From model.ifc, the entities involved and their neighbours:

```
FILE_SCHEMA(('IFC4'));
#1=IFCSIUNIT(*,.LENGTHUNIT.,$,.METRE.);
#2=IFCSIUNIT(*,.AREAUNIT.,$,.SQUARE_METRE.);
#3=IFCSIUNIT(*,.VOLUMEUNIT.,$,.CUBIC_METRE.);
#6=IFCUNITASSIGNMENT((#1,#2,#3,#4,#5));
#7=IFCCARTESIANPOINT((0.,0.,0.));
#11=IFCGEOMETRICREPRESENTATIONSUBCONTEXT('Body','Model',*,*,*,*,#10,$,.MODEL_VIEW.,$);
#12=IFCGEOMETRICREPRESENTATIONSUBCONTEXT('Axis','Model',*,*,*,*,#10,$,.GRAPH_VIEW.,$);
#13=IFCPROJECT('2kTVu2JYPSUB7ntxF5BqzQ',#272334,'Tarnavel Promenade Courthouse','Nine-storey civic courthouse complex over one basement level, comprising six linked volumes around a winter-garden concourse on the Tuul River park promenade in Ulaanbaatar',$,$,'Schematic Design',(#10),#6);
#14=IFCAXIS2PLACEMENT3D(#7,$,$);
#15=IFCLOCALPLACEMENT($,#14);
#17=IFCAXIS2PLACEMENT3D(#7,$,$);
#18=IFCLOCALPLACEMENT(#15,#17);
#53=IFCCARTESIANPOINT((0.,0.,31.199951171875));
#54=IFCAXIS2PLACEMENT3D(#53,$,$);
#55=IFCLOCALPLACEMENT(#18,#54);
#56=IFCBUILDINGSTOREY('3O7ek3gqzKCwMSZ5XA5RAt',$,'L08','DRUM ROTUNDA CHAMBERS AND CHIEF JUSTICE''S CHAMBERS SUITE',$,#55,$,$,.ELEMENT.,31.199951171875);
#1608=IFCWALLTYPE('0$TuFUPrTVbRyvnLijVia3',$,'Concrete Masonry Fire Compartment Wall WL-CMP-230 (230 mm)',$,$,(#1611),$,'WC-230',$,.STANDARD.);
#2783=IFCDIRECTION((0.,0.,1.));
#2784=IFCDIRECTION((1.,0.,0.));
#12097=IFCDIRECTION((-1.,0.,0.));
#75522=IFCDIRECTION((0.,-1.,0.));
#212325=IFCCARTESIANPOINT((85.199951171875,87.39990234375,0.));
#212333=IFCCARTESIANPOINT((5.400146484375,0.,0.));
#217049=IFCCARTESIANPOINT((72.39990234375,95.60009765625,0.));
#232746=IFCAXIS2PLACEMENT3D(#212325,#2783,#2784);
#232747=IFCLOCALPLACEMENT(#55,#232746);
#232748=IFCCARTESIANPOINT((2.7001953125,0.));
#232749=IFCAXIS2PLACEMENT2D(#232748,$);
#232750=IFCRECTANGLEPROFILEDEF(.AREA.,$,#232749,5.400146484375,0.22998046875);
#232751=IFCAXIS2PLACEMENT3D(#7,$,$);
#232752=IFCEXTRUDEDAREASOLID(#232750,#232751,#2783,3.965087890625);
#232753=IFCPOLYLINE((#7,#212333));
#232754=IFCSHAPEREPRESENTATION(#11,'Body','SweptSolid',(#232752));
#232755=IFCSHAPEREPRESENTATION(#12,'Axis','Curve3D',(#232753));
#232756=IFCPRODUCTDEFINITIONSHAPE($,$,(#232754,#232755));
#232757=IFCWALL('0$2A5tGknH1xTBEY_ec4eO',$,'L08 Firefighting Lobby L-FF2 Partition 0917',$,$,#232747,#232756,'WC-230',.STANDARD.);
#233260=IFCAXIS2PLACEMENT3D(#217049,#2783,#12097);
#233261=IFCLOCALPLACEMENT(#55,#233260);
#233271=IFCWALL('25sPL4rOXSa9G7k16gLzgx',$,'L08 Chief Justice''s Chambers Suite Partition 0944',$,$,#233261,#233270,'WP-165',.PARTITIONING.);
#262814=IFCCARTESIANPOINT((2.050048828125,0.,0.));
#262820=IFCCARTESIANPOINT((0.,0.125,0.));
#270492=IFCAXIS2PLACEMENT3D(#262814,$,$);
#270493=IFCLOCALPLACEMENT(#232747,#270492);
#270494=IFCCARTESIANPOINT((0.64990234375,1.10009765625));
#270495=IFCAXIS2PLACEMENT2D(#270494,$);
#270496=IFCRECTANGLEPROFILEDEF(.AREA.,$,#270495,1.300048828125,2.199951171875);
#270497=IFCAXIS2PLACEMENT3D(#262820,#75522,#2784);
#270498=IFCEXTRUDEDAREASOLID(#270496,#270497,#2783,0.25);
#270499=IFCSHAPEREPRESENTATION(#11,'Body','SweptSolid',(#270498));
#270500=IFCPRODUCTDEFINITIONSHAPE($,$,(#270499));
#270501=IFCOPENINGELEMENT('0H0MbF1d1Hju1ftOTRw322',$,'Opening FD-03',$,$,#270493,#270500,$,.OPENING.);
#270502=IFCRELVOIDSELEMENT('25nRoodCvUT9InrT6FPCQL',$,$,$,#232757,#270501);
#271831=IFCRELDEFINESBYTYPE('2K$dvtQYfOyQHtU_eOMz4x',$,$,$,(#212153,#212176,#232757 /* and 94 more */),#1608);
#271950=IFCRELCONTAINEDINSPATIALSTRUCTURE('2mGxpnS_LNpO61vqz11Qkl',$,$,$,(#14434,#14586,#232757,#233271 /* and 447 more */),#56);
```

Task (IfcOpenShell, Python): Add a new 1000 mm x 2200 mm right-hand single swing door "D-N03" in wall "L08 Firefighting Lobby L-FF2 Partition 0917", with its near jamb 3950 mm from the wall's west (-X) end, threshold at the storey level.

```python
import numpy as np
import ifcopenshell
import ifcopenshell.api.feature
import ifcopenshell.api.geometry
import ifcopenshell.api.root
import ifcopenshell.api.spatial
import ifcopenshell.geom
import ifcopenshell.util.element
import ifcopenshell.util.placement
import ifcopenshell.util.representation
import ifcopenshell.util.shape
import ifcopenshell.util.unit

model = ifcopenshell.open("model.ifc")
unit_scale = ifcopenshell.util.unit.calculate_unit_scale(model)
settings = ifcopenshell.geom.settings()


def volume(element):
    """Net volume in cubic metres, openings subtracted."""
    shape = ifcopenshell.geom.create_shape(settings, element)
    return ifcopenshell.util.shape.get_volume(shape.geometry)


wall = model.by_id(232757)
storey = ifcopenshell.util.element.get_container(wall, ifc_class="IfcBuildingStorey")
context = ifcopenshell.util.representation.get_context(model, "Model", "Body", "MODEL_VIEW")
before = volume(wall)

width, height, from_end, sill = 1, 2.2, 3.95, 0.0  # metres

# The wall runs along its own X axis, and the end named is its -X end.
wall_shape = ifcopenshell.geom.create_shape(settings, wall)
x, y, z = ifcopenshell.util.shape.get_vertices(wall_shape.geometry).T
start = x.min() + from_end
face, thickness = float(y.min()), float(y.max() - y.min())
wall_matrix = ifcopenshell.util.placement.get_local_placement(wall.ObjectPlacement)
level = ifcopenshell.util.placement.get_local_placement(storey.ObjectPlacement)[2, 3]


def in_wall(x, y):
    """Placement at x, y metres in the wall's axes, at sill height."""
    matrix = wall_matrix.copy()
    matrix[:, 3] = wall_matrix @ np.array([x / unit_scale, y / unit_scale, 0.0, 1.0])
    matrix[2, 3] = level + sill / unit_scale
    return matrix


# Opening: a box that overshoots both wall faces by 50 mm.
opening = ifcopenshell.api.root.create_entity(model, ifc_class="IfcOpeningElement", predefined_type="OPENING")
box = ifcopenshell.api.geometry.add_wall_representation(
    model, context=context, length=width, height=height, thickness=thickness + 0.1
)
ifcopenshell.api.geometry.assign_representation(model, product=opening, representation=box)
ifcopenshell.api.geometry.edit_object_placement(model, product=opening, matrix=in_wall(start, face - 0.05), is_si=False)
ifcopenshell.api.feature.add_feature(model, feature=opening, element=wall)

door = ifcopenshell.api.root.create_entity(model, ifc_class="IfcDoor", name="D-N03", predefined_type="DOOR")
door.OverallWidth, door.OverallHeight = width / unit_scale, height / unit_scale
door.OperationType = "SINGLE_SWING_RIGHT"
body = ifcopenshell.api.geometry.add_door_representation(
    model,
    context=context,
    overall_width=door.OverallWidth,
    overall_height=door.OverallHeight,
    operation_type="SINGLE_SWING_RIGHT",
    lining_properties={"LiningDepth": thickness / unit_scale, "ThresholdDepth": thickness / unit_scale},
)
ifcopenshell.api.geometry.assign_representation(model, product=door, representation=body)
ifcopenshell.api.spatial.assign_container(model, products=[door], relating_structure=storey)
ifcopenshell.api.feature.add_filling(model, opening=opening, element=door)

# The lining spans the wall, so the door starts at the wall face.
ifcopenshell.api.geometry.edit_object_placement(model, product=door, matrix=in_wall(start, face), is_si=False)

after = volume(wall)

print(f"wall volume {before:.3f} -> {after:.3f} m3")

model.write("model_edited.ifc")
```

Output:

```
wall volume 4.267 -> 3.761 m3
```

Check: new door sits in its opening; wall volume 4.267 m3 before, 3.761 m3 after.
